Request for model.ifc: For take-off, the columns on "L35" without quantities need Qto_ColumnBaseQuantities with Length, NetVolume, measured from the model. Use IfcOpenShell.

First a look at what the model holds.

```python
import ifcopenshell
import ifcopenshell.util.element
import ifcopenshell.util.unit

model = ifcopenshell.open("model.ifc")
print(model.schema)
for unit_type in ("LENGTHUNIT", "AREAUNIT", "VOLUMEUNIT"):
    print(unit_type, ifcopenshell.util.unit.calculate_unit_scale(model, unit_type))
storey = next(s for s in model.by_type("IfcBuildingStorey") if s.Name == "L35")
columns = [e for e in ifcopenshell.util.element.get_decomposition(storey) if e.is_a("IfcColumn")]
for e in sorted(columns, key=lambda e: e.id()):
    print(e.id(), e.is_a(), e.Name, list(ifcopenshell.util.element.get_psets(e, qtos_only=True)), sep=" | ")
```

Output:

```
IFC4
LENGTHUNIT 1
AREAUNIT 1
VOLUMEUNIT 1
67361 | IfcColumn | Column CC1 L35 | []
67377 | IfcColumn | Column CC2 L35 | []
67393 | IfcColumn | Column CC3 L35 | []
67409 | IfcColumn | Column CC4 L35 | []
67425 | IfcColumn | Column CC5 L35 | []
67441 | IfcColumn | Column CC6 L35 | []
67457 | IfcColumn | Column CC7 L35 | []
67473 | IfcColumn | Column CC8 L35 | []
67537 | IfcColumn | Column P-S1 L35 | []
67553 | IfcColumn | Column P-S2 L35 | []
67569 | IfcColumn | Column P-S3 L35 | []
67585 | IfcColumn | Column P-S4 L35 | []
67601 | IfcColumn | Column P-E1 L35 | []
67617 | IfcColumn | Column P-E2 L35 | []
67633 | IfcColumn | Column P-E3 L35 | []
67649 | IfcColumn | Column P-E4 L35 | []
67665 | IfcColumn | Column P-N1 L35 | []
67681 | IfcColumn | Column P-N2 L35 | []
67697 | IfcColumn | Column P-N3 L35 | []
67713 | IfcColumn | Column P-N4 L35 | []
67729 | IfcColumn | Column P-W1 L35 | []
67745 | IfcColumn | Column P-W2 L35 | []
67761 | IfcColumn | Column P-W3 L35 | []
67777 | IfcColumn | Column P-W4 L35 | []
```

```python
import ifcopenshell
import ifcopenshell.api.pset
import ifcopenshell.geom
import ifcopenshell.util.element
import ifcopenshell.util.shape
import ifcopenshell.util.unit

model = ifcopenshell.open("model.ifc")
unit_scale = ifcopenshell.util.unit.calculate_unit_scale(model)
volume_scale = ifcopenshell.util.unit.calculate_unit_scale(model, "VOLUMEUNIT")
settings = ifcopenshell.geom.settings()

storey = next(s for s in model.by_type("IfcBuildingStorey") if s.Name == "L35")
columns = [e for e in ifcopenshell.util.element.get_decomposition(storey) if e.is_a("IfcColumn")]

for e in sorted(columns, key=lambda e: e.id()):
    if ifcopenshell.util.element.get_psets(e, qtos_only=True, should_inherit=False):
        continue
    # Geometry comes back in metres, in the element's own axes.
    shape = ifcopenshell.geom.create_shape(settings, e)
    values = {
        "Length": ifcopenshell.util.shape.get_z(shape.geometry) / unit_scale,
        "NetVolume": ifcopenshell.util.shape.get_volume(shape.geometry) / volume_scale,
    }
    qto = ifcopenshell.api.pset.add_qto(model, product=e, name="Qto_ColumnBaseQuantities")
    ifcopenshell.api.pset.edit_qto(model, qto=qto, properties=values)
    print(e.id(), {k: round(v, 3) for k, v in values.items()})

model.write("model_updated.ifc")
```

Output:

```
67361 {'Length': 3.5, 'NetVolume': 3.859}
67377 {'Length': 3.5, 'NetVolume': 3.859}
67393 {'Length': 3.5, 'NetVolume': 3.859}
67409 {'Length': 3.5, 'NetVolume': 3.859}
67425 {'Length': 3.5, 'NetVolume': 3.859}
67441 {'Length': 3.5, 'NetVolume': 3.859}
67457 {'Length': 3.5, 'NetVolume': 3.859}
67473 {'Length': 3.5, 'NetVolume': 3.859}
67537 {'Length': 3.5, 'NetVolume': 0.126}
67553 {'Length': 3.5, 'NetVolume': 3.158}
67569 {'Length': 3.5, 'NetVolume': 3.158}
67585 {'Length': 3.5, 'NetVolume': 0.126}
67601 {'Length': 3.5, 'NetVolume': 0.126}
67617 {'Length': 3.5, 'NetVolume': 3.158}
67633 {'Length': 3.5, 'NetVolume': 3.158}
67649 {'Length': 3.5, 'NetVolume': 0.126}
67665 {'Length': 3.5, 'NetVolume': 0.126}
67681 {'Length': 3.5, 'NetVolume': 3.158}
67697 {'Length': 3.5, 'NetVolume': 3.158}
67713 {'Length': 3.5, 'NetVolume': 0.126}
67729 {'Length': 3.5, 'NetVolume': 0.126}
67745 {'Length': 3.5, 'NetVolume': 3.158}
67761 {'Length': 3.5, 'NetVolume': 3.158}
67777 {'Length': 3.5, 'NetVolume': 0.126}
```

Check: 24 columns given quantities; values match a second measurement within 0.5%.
